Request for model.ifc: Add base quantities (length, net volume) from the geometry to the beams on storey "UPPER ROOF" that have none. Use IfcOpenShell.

First a look at what the model holds.

```python
import ifcopenshell
import ifcopenshell.util.element
import ifcopenshell.util.unit

model = ifcopenshell.open("model.ifc")
print(model.schema)
for unit_type in ("LENGTHUNIT", "AREAUNIT", "VOLUMEUNIT"):
    print(unit_type, ifcopenshell.util.unit.calculate_unit_scale(model, unit_type))
storey = next(s for s in model.by_type("IfcBuildingStorey") if s.Name == "UPPER ROOF")
beams = [e for e in ifcopenshell.util.element.get_decomposition(storey) if e.is_a("IfcBeam")]
for e in sorted(beams, key=lambda e: e.id()):
    print(e.id(), e.is_a(), e.Name, list(ifcopenshell.util.element.get_psets(e, qtos_only=True)), sep=" | ")
```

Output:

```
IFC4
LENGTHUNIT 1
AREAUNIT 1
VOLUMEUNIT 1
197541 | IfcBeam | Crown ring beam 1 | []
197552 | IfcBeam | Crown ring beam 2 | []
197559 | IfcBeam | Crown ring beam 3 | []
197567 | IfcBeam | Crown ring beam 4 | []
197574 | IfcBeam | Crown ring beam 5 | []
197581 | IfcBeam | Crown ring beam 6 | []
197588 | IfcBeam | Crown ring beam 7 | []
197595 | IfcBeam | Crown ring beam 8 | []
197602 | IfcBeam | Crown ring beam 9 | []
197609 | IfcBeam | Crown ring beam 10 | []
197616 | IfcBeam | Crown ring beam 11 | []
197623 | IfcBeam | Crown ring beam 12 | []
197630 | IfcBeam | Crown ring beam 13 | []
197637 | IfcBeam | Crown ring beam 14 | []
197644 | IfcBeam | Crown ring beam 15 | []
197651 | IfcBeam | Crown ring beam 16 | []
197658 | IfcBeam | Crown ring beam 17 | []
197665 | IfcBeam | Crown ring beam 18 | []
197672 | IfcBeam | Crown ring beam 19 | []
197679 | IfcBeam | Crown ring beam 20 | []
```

```python
import ifcopenshell
import ifcopenshell.api.pset
import ifcopenshell.geom
import ifcopenshell.util.element
import ifcopenshell.util.shape
import ifcopenshell.util.unit

model = ifcopenshell.open("model.ifc")
unit_scale = ifcopenshell.util.unit.calculate_unit_scale(model)
volume_scale = ifcopenshell.util.unit.calculate_unit_scale(model, "VOLUMEUNIT")
settings = ifcopenshell.geom.settings()

storey = next(s for s in model.by_type("IfcBuildingStorey") if s.Name == "UPPER ROOF")
beams = [e for e in ifcopenshell.util.element.get_decomposition(storey) if e.is_a("IfcBeam")]

for e in sorted(beams, key=lambda e: e.id()):
    if ifcopenshell.util.element.get_psets(e, qtos_only=True, should_inherit=False):
        continue
    # Geometry comes back in metres, in the element's own axes.
    shape = ifcopenshell.geom.create_shape(settings, e)
    values = {
        "Length": ifcopenshell.util.shape.get_max_xyz(shape.geometry) / unit_scale,
        "NetVolume": ifcopenshell.util.shape.get_volume(shape.geometry) / volume_scale,
    }
    qto = ifcopenshell.api.pset.add_qto(model, product=e, name="Qto_BeamBaseQuantities")
    ifcopenshell.api.pset.edit_qto(model, qto=qto, properties=values)
    print(e.id(), {k: round(v, 3) for k, v in values.items()})

model.write("model-out.ifc")
```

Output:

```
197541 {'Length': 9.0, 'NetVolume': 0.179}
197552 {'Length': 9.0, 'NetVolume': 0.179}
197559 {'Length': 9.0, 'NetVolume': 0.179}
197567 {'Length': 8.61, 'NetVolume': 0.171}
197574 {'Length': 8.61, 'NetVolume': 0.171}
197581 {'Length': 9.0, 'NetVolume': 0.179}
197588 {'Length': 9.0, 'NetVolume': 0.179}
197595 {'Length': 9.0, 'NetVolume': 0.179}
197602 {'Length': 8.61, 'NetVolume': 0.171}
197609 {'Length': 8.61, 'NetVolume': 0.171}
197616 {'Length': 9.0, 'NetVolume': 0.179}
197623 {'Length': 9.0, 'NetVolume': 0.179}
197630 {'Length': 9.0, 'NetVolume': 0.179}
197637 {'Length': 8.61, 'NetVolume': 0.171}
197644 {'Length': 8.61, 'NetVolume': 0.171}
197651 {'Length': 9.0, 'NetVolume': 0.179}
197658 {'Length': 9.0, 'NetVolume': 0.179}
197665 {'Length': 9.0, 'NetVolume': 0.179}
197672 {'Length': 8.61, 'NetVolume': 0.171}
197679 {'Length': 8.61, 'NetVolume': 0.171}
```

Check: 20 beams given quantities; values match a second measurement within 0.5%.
